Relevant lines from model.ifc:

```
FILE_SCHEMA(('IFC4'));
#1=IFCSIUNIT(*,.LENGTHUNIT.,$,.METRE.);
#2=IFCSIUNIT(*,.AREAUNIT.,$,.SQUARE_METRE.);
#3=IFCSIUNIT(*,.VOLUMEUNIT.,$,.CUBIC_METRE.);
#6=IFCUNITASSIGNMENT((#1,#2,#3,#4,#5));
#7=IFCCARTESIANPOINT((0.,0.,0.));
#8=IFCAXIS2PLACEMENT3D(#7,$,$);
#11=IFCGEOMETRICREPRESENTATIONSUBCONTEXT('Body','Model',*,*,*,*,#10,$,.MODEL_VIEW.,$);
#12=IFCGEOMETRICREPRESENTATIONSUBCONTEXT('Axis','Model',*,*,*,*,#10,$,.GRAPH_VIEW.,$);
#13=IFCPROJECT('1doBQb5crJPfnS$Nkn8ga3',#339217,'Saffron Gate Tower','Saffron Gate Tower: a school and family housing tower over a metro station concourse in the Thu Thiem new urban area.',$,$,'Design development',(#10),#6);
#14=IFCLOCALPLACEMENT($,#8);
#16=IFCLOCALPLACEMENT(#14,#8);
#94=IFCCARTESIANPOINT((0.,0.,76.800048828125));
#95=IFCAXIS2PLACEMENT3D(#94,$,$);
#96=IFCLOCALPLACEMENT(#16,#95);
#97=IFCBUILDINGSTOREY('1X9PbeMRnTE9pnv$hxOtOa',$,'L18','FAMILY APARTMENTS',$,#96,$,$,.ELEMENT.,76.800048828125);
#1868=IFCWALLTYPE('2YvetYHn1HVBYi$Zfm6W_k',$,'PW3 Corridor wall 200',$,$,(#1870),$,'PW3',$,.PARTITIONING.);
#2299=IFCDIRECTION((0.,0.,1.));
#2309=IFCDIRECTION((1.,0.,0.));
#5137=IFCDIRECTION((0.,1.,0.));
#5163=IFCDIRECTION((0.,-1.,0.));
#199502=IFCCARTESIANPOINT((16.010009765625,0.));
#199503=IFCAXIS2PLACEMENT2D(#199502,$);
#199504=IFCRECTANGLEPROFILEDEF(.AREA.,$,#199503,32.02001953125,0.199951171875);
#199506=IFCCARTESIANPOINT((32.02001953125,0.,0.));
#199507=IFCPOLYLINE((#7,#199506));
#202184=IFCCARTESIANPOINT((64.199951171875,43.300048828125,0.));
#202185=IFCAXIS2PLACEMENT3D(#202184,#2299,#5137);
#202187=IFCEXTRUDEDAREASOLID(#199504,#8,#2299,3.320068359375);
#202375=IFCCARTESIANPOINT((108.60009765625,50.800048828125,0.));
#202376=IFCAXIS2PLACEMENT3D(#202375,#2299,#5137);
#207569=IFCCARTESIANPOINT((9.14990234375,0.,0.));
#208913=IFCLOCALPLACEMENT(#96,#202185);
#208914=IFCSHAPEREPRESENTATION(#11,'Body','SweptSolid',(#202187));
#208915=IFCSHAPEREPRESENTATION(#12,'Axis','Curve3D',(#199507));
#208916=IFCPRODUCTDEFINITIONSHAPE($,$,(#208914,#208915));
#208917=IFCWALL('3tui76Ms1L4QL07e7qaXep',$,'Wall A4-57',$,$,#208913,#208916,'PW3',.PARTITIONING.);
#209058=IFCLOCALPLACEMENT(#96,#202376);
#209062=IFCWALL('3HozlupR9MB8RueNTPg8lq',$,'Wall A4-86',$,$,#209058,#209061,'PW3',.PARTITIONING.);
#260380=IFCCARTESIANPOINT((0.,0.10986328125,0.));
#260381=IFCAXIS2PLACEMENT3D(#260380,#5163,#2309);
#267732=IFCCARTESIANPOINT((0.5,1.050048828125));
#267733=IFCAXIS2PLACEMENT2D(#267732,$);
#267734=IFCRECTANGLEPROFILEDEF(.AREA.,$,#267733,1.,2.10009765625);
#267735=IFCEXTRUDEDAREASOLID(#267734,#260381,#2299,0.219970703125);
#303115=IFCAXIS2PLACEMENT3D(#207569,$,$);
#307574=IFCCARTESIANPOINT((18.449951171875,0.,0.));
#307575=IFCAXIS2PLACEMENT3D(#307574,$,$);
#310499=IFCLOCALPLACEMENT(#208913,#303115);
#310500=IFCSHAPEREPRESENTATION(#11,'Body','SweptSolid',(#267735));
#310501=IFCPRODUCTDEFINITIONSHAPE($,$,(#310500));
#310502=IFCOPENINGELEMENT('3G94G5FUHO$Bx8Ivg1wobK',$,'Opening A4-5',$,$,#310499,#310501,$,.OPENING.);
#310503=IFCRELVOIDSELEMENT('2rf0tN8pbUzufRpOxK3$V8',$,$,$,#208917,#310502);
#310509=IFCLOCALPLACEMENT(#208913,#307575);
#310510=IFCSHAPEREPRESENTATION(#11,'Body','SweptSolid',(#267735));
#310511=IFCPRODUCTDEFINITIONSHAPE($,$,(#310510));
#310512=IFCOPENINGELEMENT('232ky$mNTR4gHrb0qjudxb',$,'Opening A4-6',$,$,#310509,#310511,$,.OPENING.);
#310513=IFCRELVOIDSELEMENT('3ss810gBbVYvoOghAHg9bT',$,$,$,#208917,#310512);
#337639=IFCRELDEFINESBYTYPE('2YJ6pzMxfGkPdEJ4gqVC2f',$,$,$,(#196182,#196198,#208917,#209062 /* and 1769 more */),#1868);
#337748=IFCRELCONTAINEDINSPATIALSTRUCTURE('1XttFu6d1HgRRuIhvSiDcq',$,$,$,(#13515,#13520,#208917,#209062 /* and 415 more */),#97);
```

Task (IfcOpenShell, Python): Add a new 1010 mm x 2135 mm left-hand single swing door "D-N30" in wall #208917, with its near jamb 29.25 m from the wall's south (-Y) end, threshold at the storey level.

```python
import numpy as np
import ifcopenshell
import ifcopenshell.api.feature
import ifcopenshell.api.geometry
import ifcopenshell.api.root
import ifcopenshell.api.spatial
import ifcopenshell.geom
import ifcopenshell.util.element
import ifcopenshell.util.placement
import ifcopenshell.util.representation
import ifcopenshell.util.shape
import ifcopenshell.util.unit

model = ifcopenshell.open("model.ifc")
unit_scale = ifcopenshell.util.unit.calculate_unit_scale(model)
settings = ifcopenshell.geom.settings()


def volume(element):
    """Net volume in cubic metres, openings subtracted."""
    shape = ifcopenshell.geom.create_shape(settings, element)
    return ifcopenshell.util.shape.get_volume(shape.geometry)


wall = model.by_guid("3tui76Ms1L4QL07e7qaXep")
storey = ifcopenshell.util.element.get_container(wall, ifc_class="IfcBuildingStorey")
context = ifcopenshell.util.representation.get_context(model, "Model", "Body", "MODEL_VIEW")
before = volume(wall)

width, height, from_end, sill = 1.01, 2.135, 29.25, 0.0  # metres

# The wall runs along its own X axis, and the end named is its -X end.
wall_shape = ifcopenshell.geom.create_shape(settings, wall)
x, y, z = ifcopenshell.util.shape.get_vertices(wall_shape.geometry).T
start = x.min() + from_end
face, thickness = float(y.min()), float(y.max() - y.min())
wall_matrix = ifcopenshell.util.placement.get_local_placement(wall.ObjectPlacement)
level = ifcopenshell.util.placement.get_local_placement(storey.ObjectPlacement)[2, 3]


def in_wall(x, y):
    """Placement at x, y metres in the wall's axes, at sill height."""
    matrix = wall_matrix.copy()
    matrix[:, 3] = wall_matrix @ np.array([x / unit_scale, y / unit_scale, 0.0, 1.0])
    matrix[2, 3] = level + sill / unit_scale
    return matrix


# Opening: a box that overshoots both wall faces by 50 mm.
opening = ifcopenshell.api.root.create_entity(model, ifc_class="IfcOpeningElement", predefined_type="OPENING")
box = ifcopenshell.api.geometry.add_wall_representation(
    model, context=context, length=width, height=height, thickness=thickness + 0.1
)
ifcopenshell.api.geometry.assign_representation(model, product=opening, representation=box)
ifcopenshell.api.geometry.edit_object_placement(model, product=opening, matrix=in_wall(start, face - 0.05), is_si=False)
ifcopenshell.api.feature.add_feature(model, feature=opening, element=wall)

door = ifcopenshell.api.root.create_entity(model, ifc_class="IfcDoor", name="D-N30", predefined_type="DOOR")
door.OverallWidth, door.OverallHeight = width / unit_scale, height / unit_scale
door.OperationType = "SINGLE_SWING_LEFT"
body = ifcopenshell.api.geometry.add_door_representation(
    model,
    context=context,
    overall_width=door.OverallWidth,
    overall_height=door.OverallHeight,
    operation_type="SINGLE_SWING_LEFT",
    lining_properties={"LiningDepth": thickness / unit_scale, "ThresholdDepth": thickness / unit_scale},
)
ifcopenshell.api.geometry.assign_representation(model, product=door, representation=body)
ifcopenshell.api.spatial.assign_container(model, products=[door], relating_structure=storey)
ifcopenshell.api.feature.add_filling(model, opening=opening, element=door)

# The lining spans the wall, so the door starts at the wall face.
ifcopenshell.api.geometry.edit_object_placement(model, product=door, matrix=in_wall(start, face), is_si=False)

after = volume(wall)

print(f"wall volume {before:.3f} -> {after:.3f} m3")

model.write("model-out.ifc")
```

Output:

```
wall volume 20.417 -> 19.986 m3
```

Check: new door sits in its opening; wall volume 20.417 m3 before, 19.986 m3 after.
